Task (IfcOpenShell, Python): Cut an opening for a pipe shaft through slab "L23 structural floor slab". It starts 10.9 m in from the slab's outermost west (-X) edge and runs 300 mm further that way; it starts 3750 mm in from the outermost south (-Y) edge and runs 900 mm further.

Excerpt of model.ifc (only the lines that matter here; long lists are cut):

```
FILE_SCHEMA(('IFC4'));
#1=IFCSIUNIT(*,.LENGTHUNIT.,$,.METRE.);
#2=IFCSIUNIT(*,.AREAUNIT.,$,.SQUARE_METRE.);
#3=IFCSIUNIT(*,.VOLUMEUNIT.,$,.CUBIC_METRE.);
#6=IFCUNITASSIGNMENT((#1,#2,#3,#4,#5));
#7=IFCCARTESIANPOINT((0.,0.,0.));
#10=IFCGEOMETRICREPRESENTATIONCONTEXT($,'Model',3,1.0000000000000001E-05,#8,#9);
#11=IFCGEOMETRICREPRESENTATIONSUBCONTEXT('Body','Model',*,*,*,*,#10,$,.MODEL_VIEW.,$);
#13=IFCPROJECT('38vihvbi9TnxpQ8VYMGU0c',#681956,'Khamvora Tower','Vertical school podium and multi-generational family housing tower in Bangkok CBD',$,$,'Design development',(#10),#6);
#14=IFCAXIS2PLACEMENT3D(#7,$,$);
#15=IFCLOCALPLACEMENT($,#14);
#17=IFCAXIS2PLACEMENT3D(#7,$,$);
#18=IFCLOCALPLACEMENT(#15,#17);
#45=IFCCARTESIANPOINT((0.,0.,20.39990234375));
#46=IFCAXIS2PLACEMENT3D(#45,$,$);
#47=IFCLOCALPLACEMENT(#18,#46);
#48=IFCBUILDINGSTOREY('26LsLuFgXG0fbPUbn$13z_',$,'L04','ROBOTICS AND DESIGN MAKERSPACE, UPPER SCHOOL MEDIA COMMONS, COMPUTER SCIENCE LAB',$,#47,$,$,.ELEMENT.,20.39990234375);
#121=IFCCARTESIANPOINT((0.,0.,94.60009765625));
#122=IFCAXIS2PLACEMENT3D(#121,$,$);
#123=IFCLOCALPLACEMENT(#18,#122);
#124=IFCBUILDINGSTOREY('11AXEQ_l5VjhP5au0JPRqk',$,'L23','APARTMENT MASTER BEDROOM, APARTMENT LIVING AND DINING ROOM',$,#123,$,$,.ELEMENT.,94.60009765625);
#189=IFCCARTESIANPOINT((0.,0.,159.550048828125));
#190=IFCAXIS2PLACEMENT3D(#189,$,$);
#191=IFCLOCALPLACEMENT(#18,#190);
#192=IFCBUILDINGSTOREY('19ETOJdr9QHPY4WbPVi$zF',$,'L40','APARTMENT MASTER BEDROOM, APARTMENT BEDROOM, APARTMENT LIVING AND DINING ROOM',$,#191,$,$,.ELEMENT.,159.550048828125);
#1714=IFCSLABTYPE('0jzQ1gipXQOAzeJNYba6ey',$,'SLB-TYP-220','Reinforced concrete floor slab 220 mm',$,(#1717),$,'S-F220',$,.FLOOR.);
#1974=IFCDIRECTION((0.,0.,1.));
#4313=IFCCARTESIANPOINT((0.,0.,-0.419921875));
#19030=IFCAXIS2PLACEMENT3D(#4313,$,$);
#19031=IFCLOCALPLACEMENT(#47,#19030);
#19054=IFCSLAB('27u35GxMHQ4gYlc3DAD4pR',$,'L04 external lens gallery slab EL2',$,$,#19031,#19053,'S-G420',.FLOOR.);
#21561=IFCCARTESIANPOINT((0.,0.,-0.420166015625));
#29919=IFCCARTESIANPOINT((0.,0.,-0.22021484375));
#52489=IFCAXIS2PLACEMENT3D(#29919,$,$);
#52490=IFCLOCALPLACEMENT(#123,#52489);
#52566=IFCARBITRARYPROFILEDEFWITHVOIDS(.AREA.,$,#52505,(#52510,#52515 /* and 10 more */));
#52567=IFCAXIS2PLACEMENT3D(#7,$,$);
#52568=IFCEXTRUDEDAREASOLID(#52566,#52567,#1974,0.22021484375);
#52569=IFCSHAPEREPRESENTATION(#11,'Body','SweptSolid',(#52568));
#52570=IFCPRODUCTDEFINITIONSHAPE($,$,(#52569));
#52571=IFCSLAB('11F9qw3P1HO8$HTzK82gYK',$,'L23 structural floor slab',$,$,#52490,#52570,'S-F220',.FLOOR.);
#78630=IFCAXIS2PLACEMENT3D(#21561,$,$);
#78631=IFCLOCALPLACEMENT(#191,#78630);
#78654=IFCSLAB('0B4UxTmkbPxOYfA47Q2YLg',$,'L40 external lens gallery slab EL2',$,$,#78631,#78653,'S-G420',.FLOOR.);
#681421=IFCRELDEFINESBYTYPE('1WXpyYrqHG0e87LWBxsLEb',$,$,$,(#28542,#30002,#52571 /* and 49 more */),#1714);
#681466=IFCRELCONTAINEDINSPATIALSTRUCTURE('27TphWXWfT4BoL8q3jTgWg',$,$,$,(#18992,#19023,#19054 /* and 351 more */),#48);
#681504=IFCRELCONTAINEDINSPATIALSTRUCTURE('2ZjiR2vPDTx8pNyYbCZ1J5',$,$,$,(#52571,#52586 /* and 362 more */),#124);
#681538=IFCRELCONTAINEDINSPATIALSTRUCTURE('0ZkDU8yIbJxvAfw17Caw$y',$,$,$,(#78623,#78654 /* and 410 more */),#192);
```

```python
import numpy as np
import ifcopenshell
import ifcopenshell.api.feature
import ifcopenshell.api.geometry
import ifcopenshell.api.root
import ifcopenshell.geom
import ifcopenshell.util.placement
import ifcopenshell.util.representation
import ifcopenshell.util.shape
import ifcopenshell.util.unit

model = ifcopenshell.open("model.ifc")
unit_scale = ifcopenshell.util.unit.calculate_unit_scale(model)
settings = ifcopenshell.geom.settings()


def volume(element):
    """Net volume in cubic metres, openings subtracted."""
    shape = ifcopenshell.geom.create_shape(settings, element)
    return ifcopenshell.util.shape.get_volume(shape.geometry)


slab = model.by_id(52571)
before = volume(slab)

# Extent in the slab's own axes, in metres. The edges named are its -X and -Y sides.
slab_shape = ifcopenshell.geom.create_shape(settings, slab)
vertices = ifcopenshell.util.shape.get_vertices(slab_shape.geometry)
x_min, y_min, bottom = vertices.min(axis=0)
top = vertices[:, 2].max()

opening = ifcopenshell.api.root.create_entity(model, ifc_class="IfcOpeningElement", name="Pipe shaft opening", predefined_type="OPENING")
context = ifcopenshell.util.representation.get_context(model, "Model", "Body", "MODEL_VIEW")
width, depth = 0.3, 0.9
outline = [(0.0, 0.0), (width, 0.0), (width, depth), (0.0, depth), (0.0, 0.0)]
# Overshoot both faces by 50 mm so the cut is clean.
shape = ifcopenshell.api.geometry.add_slab_representation(
    model, context=context, depth=top - bottom + 0.1, polyline=outline
)
ifcopenshell.api.geometry.assign_representation(model, product=opening, representation=shape)

matrix = ifcopenshell.util.placement.get_local_placement(slab.ObjectPlacement)
matrix[:, 3] = matrix @ np.append(np.array([x_min + 10.9, y_min + 3.75, bottom - 0.05]) / unit_scale, 1.0)
ifcopenshell.api.geometry.edit_object_placement(model, product=opening, matrix=matrix, is_si=False)
ifcopenshell.api.feature.add_feature(model, feature=opening, element=slab)

after = volume(slab)

print(f"slab volume {before:.3f} -> {after:.3f} m3")

model.write("model_updated.ifc")
```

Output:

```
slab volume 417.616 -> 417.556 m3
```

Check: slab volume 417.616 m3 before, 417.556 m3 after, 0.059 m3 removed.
